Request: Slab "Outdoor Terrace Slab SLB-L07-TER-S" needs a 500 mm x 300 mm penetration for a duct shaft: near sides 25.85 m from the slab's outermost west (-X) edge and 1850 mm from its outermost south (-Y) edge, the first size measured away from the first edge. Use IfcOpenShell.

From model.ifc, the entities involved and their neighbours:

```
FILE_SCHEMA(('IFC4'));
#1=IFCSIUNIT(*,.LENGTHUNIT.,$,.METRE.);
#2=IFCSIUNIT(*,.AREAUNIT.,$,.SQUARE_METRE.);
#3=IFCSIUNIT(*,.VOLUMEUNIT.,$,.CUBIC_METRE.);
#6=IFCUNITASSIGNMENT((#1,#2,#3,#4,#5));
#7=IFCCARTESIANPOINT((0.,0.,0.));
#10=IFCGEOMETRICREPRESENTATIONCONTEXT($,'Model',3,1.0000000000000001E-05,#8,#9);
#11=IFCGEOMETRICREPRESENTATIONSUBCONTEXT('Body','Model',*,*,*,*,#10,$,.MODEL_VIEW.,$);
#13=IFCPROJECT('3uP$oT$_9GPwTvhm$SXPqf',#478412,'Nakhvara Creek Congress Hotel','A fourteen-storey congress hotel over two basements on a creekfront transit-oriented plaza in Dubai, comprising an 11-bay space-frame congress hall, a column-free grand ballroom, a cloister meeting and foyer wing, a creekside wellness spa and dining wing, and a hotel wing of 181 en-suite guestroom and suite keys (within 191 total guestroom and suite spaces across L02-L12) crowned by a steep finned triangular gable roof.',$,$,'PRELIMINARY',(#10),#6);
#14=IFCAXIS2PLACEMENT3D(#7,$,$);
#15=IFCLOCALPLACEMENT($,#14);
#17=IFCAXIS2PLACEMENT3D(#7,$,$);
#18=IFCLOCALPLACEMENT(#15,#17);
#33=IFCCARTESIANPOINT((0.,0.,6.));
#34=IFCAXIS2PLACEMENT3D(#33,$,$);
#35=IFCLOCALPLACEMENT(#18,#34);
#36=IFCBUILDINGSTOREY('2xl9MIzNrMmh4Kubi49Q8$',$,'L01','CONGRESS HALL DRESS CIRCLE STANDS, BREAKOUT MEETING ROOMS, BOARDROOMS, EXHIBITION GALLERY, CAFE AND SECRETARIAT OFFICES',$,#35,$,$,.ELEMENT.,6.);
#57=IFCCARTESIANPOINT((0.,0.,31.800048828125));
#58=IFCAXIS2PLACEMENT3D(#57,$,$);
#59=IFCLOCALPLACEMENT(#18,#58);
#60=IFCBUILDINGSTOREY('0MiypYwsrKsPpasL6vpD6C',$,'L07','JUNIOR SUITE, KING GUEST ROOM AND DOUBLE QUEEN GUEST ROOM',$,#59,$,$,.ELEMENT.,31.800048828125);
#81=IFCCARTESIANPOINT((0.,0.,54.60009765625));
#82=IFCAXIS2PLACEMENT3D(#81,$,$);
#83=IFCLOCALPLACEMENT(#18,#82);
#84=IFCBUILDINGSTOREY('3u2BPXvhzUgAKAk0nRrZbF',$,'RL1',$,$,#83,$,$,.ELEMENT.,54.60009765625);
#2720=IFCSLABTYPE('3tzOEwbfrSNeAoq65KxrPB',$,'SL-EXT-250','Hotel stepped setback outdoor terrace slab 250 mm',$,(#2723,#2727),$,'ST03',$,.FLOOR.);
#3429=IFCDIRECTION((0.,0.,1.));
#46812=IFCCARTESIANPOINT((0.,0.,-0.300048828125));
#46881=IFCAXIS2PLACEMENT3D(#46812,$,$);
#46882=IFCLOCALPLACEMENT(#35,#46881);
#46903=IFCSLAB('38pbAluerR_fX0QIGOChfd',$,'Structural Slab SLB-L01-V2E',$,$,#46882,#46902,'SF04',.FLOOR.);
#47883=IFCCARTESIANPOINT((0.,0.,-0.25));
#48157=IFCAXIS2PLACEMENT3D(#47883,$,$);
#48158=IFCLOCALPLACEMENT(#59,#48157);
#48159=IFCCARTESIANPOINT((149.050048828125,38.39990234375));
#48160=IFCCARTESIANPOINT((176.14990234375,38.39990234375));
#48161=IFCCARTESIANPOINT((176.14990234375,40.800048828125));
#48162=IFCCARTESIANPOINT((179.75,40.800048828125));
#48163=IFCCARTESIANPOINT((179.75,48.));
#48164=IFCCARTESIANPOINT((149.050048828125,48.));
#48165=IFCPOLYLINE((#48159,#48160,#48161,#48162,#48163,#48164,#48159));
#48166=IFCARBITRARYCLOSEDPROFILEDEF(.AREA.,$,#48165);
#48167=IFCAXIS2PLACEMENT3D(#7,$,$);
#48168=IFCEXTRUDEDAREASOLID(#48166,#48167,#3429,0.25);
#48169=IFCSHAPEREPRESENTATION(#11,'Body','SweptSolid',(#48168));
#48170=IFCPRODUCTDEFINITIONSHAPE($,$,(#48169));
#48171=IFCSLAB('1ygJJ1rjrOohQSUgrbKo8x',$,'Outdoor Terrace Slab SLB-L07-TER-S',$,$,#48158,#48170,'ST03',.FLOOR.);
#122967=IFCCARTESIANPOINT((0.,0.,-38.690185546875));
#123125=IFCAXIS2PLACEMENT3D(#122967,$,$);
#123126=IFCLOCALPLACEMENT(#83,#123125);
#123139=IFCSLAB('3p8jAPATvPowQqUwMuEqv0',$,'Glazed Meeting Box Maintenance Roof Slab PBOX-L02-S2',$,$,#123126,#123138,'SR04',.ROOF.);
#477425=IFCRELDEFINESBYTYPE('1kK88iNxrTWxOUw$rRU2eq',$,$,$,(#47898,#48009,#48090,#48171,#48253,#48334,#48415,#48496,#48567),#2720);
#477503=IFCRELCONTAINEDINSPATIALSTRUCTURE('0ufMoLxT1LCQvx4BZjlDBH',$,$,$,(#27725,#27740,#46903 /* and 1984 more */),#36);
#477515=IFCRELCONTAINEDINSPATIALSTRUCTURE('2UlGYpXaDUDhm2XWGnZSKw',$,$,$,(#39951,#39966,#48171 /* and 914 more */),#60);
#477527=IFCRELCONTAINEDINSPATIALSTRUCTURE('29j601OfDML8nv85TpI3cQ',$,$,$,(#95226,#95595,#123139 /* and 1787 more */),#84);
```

```python
import numpy as np
import ifcopenshell
import ifcopenshell.api.feature
import ifcopenshell.api.geometry
import ifcopenshell.api.root
import ifcopenshell.geom
import ifcopenshell.util.placement
import ifcopenshell.util.representation
import ifcopenshell.util.shape
import ifcopenshell.util.unit

model = ifcopenshell.open("model.ifc")
unit_scale = ifcopenshell.util.unit.calculate_unit_scale(model)
settings = ifcopenshell.geom.settings()


def volume(element):
    """Net volume in cubic metres, openings subtracted."""
    shape = ifcopenshell.geom.create_shape(settings, element)
    return ifcopenshell.util.shape.get_volume(shape.geometry)


slab = model.by_guid("1ygJJ1rjrOohQSUgrbKo8x")
before = volume(slab)

# Extent in the slab's own axes, in metres. The edges named are its -X and -Y sides.
slab_shape = ifcopenshell.geom.create_shape(settings, slab)
vertices = ifcopenshell.util.shape.get_vertices(slab_shape.geometry)
x_min, y_min, bottom = vertices.min(axis=0)
top = vertices[:, 2].max()

opening = ifcopenshell.api.root.create_entity(model, ifc_class="IfcOpeningElement", name="Duct shaft opening", predefined_type="OPENING")
context = ifcopenshell.util.representation.get_context(model, "Model", "Body", "MODEL_VIEW")
width, depth = 0.5, 0.3
outline = [(0.0, 0.0), (width, 0.0), (width, depth), (0.0, depth), (0.0, 0.0)]
# Overshoot both faces by 50 mm so the cut is clean.
shape = ifcopenshell.api.geometry.add_slab_representation(
    model, context=context, depth=top - bottom + 0.1, polyline=outline
)
ifcopenshell.api.geometry.assign_representation(model, product=opening, representation=shape)

matrix = ifcopenshell.util.placement.get_local_placement(slab.ObjectPlacement)
matrix[:, 3] = matrix @ np.append(np.array([x_min + 25.85, y_min + 1.85, bottom - 0.05]) / unit_scale, 1.0)
ifcopenshell.api.geometry.edit_object_placement(model, product=opening, matrix=matrix, is_si=False)
ifcopenshell.api.feature.add_feature(model, feature=opening, element=slab)

after = volume(slab)

print(f"slab volume {before:.3f} -> {after:.3f} m3")

model.write("model_rev.ifc")
```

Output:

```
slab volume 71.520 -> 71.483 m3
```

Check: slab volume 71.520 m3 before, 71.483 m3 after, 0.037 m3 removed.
